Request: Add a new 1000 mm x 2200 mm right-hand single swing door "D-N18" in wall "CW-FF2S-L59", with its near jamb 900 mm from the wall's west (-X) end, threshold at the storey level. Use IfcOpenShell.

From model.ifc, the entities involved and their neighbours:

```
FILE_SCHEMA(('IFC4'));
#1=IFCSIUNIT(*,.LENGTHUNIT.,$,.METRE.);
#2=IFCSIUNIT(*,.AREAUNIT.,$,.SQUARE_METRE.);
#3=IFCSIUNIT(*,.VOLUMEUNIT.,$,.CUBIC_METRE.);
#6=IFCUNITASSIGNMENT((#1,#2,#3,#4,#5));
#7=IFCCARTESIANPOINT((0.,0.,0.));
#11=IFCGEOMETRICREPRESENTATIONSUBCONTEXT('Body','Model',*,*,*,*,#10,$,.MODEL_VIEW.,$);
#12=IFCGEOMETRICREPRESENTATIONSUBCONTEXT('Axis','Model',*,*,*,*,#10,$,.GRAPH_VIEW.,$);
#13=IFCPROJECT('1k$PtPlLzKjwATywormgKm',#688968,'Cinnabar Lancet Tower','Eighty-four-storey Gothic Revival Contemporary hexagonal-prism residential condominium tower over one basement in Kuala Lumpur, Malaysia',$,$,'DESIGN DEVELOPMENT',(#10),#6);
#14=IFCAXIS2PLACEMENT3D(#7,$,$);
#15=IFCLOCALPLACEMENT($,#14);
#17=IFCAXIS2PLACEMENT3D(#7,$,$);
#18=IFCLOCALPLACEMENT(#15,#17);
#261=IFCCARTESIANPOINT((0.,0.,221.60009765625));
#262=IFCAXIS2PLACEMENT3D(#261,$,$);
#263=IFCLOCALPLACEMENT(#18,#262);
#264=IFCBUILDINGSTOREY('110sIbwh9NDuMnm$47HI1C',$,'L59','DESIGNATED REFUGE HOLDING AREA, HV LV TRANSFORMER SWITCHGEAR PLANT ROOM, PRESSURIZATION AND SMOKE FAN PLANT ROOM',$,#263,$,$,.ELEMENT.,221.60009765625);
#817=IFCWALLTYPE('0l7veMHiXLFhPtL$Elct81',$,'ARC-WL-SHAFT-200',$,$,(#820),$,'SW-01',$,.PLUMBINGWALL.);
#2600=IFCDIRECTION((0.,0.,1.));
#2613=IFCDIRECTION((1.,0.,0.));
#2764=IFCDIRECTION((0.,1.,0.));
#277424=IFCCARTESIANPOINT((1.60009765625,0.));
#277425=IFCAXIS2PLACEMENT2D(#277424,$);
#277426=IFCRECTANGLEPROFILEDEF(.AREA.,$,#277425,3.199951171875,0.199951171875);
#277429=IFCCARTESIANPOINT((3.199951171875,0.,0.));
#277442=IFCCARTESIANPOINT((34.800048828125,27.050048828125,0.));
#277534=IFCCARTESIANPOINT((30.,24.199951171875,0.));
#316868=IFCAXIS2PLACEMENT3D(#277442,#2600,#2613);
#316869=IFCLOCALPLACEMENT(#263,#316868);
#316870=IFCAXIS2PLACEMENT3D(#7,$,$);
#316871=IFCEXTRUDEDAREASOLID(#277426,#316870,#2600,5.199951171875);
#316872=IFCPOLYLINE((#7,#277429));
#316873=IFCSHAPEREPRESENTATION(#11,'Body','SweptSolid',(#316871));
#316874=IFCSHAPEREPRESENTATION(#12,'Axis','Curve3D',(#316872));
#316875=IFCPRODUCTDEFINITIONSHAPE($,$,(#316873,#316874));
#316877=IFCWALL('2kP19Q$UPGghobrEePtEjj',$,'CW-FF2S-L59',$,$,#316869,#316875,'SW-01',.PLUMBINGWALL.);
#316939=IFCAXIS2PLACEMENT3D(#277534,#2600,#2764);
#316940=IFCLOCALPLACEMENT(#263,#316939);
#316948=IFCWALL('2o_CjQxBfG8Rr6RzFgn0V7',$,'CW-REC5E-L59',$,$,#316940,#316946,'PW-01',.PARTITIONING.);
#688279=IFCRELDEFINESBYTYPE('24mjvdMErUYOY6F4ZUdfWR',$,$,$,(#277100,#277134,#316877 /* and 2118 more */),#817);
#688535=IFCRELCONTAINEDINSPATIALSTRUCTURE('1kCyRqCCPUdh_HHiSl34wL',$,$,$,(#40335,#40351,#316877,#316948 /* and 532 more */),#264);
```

```python
import numpy as np
import ifcopenshell
import ifcopenshell.api.feature
import ifcopenshell.api.geometry
import ifcopenshell.api.root
import ifcopenshell.api.spatial
import ifcopenshell.geom
import ifcopenshell.util.element
import ifcopenshell.util.placement
import ifcopenshell.util.representation
import ifcopenshell.util.shape
import ifcopenshell.util.unit

model = ifcopenshell.open("model.ifc")
unit_scale = ifcopenshell.util.unit.calculate_unit_scale(model)
settings = ifcopenshell.geom.settings()


def volume(element):
    """Net volume in cubic metres, openings subtracted."""
    shape = ifcopenshell.geom.create_shape(settings, element)
    return ifcopenshell.util.shape.get_volume(shape.geometry)


wall = model.by_guid("2kP19Q$UPGghobrEePtEjj")
storey = ifcopenshell.util.element.get_container(wall, ifc_class="IfcBuildingStorey")
context = ifcopenshell.util.representation.get_context(model, "Model", "Body", "MODEL_VIEW")
before = volume(wall)

width, height, from_end, sill = 1, 2.2, 0.9, 0.0  # metres

# The wall runs along its own X axis, and the end named is its -X end.
wall_shape = ifcopenshell.geom.create_shape(settings, wall)
x, y, z = ifcopenshell.util.shape.get_vertices(wall_shape.geometry).T
start = x.min() + from_end
face, thickness = float(y.min()), float(y.max() - y.min())
wall_matrix = ifcopenshell.util.placement.get_local_placement(wall.ObjectPlacement)
level = ifcopenshell.util.placement.get_local_placement(storey.ObjectPlacement)[2, 3]


def in_wall(x, y):
    """Placement at x, y metres in the wall's axes, at sill height."""
    matrix = wall_matrix.copy()
    matrix[:, 3] = wall_matrix @ np.array([x / unit_scale, y / unit_scale, 0.0, 1.0])
    matrix[2, 3] = level + sill / unit_scale
    return matrix


# Opening: a box that overshoots both wall faces by 50 mm.
opening = ifcopenshell.api.root.create_entity(model, ifc_class="IfcOpeningElement", predefined_type="OPENING")
box = ifcopenshell.api.geometry.add_wall_representation(
    model, context=context, length=width, height=height, thickness=thickness + 0.1
)
ifcopenshell.api.geometry.assign_representation(model, product=opening, representation=box)
ifcopenshell.api.geometry.edit_object_placement(model, product=opening, matrix=in_wall(start, face - 0.05), is_si=False)
ifcopenshell.api.feature.add_feature(model, feature=opening, element=wall)

door = ifcopenshell.api.root.create_entity(model, ifc_class="IfcDoor", name="D-N18", predefined_type="DOOR")
door.OverallWidth, door.OverallHeight = width / unit_scale, height / unit_scale
door.OperationType = "SINGLE_SWING_RIGHT"
body = ifcopenshell.api.geometry.add_door_representation(
    model,
    context=context,
    overall_width=door.OverallWidth,
    overall_height=door.OverallHeight,
    operation_type="SINGLE_SWING_RIGHT",
    lining_properties={"LiningDepth": thickness / unit_scale, "ThresholdDepth": thickness / unit_scale},
)
ifcopenshell.api.geometry.assign_representation(model, product=door, representation=body)
ifcopenshell.api.spatial.assign_container(model, products=[door], relating_structure=storey)
ifcopenshell.api.feature.add_filling(model, opening=opening, element=door)

# The lining spans the wall, so the door starts at the wall face.
ifcopenshell.api.geometry.edit_object_placement(model, product=door, matrix=in_wall(start, face), is_si=False)

after = volume(wall)

print(f"wall volume {before:.3f} -> {after:.3f} m3")

model.write("model_rev.ifc")
```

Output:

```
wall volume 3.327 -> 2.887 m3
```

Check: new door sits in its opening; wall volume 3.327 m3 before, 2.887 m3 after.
